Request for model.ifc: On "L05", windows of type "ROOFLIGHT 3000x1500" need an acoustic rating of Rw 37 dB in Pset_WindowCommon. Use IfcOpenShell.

First a look at what the model holds.

```python
import ifcopenshell
import ifcopenshell.util.element

model = ifcopenshell.open("model.ifc")
print(model.schema)
storey = next(s for s in model.by_type("IfcBuildingStorey") if s.Name == "L05")
windows = [e for e in ifcopenshell.util.element.get_decomposition(storey) if e.is_a("IfcWindow")]
seen = {}
for e in windows:
    element_type = ifcopenshell.util.element.get_type(e)
    key = (element_type.Name if element_type != e and element_type else None, ifcopenshell.util.element.get_pset(e, "Pset_WindowCommon", "AcousticRating"))
    seen[key] = seen.get(key, 0) + 1
for (name, value), count in sorted(seen.items(), key=str):
    print(count, "x", name, "|", value)
```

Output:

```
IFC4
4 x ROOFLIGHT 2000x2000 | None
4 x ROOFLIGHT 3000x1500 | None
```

```python
import ifcopenshell
import ifcopenshell.api.pset
import ifcopenshell.util.element

model = ifcopenshell.open("model.ifc")

storey = next(s for s in model.by_type("IfcBuildingStorey") if s.Name == "L05")
windows = [e for e in ifcopenshell.util.element.get_decomposition(storey) if e.is_a("IfcWindow")]

count = 0
for e in windows:
    element_type = ifcopenshell.util.element.get_type(e)
    if element_type in (None, e) or element_type.Name != "ROOFLIGHT 3000x1500":
        continue
    found = ifcopenshell.util.element.get_pset(e, "Pset_WindowCommon", should_inherit=False)
    if found:
        pset = model.by_id(found["id"])
        if len(ifcopenshell.util.element.get_elements_by_pset(pset)) > 1:
            pset = ifcopenshell.api.pset.unshare_pset(model, products=[e], pset=pset)[0]
    else:
        pset = ifcopenshell.api.pset.add_pset(model, product=e, name="Pset_WindowCommon")
    ifcopenshell.api.pset.edit_pset(model, pset=pset, properties={"AcousticRating": "Rw 37 dB"})
    count += 1

print(count, "windows updated")

model.write("model_rev.ifc")
```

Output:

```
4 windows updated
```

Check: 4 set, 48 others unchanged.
